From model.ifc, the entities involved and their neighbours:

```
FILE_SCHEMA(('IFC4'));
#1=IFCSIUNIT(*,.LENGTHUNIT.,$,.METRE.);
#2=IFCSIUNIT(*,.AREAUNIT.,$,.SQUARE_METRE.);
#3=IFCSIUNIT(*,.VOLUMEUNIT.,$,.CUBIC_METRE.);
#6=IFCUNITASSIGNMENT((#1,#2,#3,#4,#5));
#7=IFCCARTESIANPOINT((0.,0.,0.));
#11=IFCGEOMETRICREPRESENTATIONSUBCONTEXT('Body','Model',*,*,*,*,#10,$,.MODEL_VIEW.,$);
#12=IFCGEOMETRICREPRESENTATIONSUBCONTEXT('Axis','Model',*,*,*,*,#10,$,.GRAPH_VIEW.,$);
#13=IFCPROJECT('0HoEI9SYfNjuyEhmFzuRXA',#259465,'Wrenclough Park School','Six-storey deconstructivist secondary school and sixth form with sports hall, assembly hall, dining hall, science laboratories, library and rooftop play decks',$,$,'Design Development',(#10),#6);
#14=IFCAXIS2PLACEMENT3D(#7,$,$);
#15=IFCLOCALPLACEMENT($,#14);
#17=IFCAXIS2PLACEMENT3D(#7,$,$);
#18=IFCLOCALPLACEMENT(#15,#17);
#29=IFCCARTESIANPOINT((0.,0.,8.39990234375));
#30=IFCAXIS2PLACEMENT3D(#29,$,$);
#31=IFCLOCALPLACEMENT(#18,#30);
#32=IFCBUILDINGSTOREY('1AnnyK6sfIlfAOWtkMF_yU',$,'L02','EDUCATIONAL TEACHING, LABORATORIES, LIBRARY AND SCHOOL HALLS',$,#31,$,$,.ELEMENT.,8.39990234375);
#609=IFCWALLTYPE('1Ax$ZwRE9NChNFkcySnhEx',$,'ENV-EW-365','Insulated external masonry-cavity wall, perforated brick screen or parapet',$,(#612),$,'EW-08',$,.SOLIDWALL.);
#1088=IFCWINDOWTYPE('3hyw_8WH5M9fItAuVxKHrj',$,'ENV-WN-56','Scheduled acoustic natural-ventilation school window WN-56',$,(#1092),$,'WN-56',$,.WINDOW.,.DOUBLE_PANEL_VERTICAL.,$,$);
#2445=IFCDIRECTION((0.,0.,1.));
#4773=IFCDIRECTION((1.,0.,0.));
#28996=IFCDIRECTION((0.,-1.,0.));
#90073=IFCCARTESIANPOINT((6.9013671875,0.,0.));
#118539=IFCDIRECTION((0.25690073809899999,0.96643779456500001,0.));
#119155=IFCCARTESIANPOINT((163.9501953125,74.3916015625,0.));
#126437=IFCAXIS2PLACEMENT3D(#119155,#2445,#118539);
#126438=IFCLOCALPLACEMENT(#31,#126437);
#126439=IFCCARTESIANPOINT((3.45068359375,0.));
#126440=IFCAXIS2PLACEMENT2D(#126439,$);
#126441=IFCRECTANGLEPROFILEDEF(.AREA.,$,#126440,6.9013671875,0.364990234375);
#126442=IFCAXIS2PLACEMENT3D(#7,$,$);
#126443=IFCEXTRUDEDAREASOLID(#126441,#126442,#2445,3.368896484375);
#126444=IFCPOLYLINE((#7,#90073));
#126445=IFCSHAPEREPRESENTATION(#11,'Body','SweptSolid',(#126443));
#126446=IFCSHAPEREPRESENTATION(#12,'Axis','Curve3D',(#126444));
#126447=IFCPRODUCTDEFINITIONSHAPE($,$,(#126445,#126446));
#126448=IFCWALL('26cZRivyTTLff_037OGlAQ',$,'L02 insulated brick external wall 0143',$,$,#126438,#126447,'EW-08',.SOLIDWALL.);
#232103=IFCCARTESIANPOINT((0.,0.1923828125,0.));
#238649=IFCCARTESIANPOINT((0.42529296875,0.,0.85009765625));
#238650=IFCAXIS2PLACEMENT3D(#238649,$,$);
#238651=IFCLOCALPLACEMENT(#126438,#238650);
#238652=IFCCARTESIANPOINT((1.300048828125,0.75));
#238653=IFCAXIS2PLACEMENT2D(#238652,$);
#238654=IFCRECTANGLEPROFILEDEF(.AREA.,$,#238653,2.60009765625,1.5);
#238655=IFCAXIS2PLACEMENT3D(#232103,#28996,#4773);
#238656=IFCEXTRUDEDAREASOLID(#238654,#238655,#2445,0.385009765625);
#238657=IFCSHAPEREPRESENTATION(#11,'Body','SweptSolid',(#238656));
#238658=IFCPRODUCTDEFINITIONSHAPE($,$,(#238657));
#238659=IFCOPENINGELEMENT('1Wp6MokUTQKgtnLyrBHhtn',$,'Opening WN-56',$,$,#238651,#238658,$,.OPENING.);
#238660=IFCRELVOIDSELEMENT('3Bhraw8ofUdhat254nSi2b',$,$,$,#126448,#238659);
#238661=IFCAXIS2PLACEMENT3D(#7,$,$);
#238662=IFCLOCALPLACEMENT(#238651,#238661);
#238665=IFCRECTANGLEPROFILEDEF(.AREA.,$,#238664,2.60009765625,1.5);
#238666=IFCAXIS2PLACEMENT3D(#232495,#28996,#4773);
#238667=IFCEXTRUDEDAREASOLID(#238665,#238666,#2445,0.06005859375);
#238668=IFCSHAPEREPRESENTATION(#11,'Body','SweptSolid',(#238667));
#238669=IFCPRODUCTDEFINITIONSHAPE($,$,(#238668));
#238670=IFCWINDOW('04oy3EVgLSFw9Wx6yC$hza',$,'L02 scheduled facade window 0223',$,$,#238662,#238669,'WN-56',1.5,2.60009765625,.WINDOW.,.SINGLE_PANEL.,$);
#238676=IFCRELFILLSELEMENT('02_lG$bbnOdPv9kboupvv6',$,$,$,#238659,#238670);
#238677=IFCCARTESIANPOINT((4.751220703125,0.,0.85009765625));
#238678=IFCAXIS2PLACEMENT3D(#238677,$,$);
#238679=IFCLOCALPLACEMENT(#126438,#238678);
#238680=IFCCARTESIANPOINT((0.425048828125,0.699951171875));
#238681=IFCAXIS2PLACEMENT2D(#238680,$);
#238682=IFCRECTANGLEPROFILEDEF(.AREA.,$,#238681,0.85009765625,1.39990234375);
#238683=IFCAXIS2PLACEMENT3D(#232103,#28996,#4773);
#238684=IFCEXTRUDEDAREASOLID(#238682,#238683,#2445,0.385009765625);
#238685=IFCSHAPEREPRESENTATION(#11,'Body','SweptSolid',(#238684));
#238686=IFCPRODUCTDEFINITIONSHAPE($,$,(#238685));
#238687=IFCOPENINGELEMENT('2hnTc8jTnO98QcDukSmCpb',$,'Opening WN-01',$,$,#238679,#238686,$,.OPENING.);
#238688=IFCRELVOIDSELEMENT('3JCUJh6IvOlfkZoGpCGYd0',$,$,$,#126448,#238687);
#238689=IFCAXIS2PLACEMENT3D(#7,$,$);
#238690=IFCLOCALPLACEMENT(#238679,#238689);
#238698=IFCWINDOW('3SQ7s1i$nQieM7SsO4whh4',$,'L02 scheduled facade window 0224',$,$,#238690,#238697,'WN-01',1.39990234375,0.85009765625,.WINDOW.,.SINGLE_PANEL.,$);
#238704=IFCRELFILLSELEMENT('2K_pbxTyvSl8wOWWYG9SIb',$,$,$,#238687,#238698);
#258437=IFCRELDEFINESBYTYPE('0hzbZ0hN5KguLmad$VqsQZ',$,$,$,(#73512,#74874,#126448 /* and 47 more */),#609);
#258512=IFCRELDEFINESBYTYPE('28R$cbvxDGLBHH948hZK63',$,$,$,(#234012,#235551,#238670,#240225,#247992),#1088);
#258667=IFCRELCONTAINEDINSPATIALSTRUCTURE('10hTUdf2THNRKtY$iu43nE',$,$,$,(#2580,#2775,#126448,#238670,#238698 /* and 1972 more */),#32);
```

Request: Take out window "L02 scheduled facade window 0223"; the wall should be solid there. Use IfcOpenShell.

```python
import ifcopenshell
import ifcopenshell.api.feature
import ifcopenshell.api.root
import ifcopenshell.geom
import ifcopenshell.util.shape

model = ifcopenshell.open("model.ifc")
settings = ifcopenshell.geom.settings()


def volume(element):
    """Net volume in cubic metres, openings subtracted."""
    shape = ifcopenshell.geom.create_shape(settings, element)
    return ifcopenshell.util.shape.get_volume(shape.geometry)


window = model.by_guid("04oy3EVgLSFw9Wx6yC$hza")
opening = window.FillsVoids[0].RelatingOpeningElement
wall = opening.VoidsElements[0].RelatingBuildingElement
before = volume(wall)

ifcopenshell.api.root.remove_product(model, product=window)
ifcopenshell.api.feature.remove_feature(model, feature=opening)

after = volume(wall)

print(f"wall volume {before:.3f} -> {after:.3f} m3")

model.write("model-out.ifc")
```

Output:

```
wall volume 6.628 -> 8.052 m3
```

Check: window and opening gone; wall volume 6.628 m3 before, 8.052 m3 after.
